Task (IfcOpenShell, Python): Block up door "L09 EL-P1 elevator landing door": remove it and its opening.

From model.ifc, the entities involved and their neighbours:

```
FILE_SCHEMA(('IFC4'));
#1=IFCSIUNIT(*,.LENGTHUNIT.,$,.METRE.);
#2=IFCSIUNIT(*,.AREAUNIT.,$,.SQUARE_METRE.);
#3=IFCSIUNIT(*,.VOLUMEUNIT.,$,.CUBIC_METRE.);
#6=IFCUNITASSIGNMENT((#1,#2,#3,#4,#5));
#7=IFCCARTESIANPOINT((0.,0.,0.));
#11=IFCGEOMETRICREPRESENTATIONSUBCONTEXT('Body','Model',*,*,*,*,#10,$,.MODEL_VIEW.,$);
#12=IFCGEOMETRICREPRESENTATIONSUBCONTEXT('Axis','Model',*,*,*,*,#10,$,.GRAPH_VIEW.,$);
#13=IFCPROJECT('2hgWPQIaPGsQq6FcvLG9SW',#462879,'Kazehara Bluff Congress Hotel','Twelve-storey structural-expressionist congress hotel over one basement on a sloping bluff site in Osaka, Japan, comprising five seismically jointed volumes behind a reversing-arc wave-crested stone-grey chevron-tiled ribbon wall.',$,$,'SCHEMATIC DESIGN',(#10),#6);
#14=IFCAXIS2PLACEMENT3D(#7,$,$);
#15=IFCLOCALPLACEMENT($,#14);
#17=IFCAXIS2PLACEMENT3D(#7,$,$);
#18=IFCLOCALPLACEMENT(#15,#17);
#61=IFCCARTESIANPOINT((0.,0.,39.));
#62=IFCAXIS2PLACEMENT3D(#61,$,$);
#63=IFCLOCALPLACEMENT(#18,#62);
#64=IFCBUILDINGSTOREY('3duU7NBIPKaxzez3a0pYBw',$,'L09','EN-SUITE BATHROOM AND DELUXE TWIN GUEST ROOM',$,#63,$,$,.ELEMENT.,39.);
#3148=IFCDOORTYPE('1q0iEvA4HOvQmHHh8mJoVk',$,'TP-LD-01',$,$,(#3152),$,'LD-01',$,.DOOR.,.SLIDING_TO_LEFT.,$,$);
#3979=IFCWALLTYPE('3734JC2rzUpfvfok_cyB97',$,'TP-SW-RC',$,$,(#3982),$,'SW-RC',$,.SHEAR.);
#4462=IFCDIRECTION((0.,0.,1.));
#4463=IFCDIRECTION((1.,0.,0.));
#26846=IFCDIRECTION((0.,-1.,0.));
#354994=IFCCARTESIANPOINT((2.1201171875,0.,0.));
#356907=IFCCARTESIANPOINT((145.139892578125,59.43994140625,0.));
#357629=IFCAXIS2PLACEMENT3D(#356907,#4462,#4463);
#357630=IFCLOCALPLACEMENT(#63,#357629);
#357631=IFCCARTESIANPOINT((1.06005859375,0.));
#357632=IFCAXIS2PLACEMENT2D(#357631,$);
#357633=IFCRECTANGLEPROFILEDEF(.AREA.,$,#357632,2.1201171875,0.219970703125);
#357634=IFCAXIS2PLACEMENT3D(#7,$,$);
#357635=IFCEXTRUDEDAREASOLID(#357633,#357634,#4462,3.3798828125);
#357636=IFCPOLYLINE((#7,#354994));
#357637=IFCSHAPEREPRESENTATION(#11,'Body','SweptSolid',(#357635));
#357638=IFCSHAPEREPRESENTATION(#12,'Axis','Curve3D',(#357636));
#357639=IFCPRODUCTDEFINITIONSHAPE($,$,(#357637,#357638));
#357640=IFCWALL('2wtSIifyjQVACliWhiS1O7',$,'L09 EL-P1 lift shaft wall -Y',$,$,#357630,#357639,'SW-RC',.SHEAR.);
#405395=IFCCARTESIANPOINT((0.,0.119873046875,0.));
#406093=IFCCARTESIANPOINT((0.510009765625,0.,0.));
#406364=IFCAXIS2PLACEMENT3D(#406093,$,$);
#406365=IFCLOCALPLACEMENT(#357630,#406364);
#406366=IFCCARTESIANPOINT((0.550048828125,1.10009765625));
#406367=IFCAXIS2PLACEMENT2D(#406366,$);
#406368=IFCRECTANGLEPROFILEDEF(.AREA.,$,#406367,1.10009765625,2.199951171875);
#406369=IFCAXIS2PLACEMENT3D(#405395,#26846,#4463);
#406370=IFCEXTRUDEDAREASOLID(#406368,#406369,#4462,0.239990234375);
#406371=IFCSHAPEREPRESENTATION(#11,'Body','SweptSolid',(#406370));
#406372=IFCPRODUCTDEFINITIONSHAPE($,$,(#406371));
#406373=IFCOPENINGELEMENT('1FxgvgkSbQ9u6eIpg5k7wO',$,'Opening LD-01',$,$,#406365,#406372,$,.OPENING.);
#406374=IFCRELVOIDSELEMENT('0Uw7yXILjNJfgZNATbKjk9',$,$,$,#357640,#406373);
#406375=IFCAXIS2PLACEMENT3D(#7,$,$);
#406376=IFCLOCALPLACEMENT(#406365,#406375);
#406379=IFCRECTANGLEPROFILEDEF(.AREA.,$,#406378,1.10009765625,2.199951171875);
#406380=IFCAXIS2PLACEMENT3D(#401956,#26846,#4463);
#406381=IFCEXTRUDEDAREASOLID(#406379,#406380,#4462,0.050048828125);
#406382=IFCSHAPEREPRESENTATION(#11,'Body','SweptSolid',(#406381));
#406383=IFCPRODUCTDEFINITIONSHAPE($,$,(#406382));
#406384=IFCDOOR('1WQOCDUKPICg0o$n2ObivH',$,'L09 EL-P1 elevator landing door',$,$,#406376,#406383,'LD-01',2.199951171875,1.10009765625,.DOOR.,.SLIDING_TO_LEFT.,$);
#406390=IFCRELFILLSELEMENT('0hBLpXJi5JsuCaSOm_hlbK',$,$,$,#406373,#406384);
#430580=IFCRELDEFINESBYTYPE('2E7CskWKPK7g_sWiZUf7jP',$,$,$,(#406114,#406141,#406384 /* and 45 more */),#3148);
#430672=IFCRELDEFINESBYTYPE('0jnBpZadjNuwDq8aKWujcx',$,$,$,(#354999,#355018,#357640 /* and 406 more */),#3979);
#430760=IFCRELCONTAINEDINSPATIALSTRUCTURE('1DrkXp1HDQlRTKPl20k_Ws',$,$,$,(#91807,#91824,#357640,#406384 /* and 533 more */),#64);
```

```python
import ifcopenshell
import ifcopenshell.api.feature
import ifcopenshell.api.root
import ifcopenshell.geom
import ifcopenshell.util.shape

model = ifcopenshell.open("model.ifc")
settings = ifcopenshell.geom.settings()


def volume(element):
    """Net volume in cubic metres, openings subtracted."""
    shape = ifcopenshell.geom.create_shape(settings, element)
    return ifcopenshell.util.shape.get_volume(shape.geometry)


door = model.by_id(406384)
opening = door.FillsVoids[0].RelatingOpeningElement
wall = opening.VoidsElements[0].RelatingBuildingElement
before = volume(wall)

ifcopenshell.api.root.remove_product(model, product=door)
ifcopenshell.api.feature.remove_feature(model, feature=opening)

after = volume(wall)

print(f"wall volume {before:.3f} -> {after:.3f} m3")

model.write("model_updated.ifc")
```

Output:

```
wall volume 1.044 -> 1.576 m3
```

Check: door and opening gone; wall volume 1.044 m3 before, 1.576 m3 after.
